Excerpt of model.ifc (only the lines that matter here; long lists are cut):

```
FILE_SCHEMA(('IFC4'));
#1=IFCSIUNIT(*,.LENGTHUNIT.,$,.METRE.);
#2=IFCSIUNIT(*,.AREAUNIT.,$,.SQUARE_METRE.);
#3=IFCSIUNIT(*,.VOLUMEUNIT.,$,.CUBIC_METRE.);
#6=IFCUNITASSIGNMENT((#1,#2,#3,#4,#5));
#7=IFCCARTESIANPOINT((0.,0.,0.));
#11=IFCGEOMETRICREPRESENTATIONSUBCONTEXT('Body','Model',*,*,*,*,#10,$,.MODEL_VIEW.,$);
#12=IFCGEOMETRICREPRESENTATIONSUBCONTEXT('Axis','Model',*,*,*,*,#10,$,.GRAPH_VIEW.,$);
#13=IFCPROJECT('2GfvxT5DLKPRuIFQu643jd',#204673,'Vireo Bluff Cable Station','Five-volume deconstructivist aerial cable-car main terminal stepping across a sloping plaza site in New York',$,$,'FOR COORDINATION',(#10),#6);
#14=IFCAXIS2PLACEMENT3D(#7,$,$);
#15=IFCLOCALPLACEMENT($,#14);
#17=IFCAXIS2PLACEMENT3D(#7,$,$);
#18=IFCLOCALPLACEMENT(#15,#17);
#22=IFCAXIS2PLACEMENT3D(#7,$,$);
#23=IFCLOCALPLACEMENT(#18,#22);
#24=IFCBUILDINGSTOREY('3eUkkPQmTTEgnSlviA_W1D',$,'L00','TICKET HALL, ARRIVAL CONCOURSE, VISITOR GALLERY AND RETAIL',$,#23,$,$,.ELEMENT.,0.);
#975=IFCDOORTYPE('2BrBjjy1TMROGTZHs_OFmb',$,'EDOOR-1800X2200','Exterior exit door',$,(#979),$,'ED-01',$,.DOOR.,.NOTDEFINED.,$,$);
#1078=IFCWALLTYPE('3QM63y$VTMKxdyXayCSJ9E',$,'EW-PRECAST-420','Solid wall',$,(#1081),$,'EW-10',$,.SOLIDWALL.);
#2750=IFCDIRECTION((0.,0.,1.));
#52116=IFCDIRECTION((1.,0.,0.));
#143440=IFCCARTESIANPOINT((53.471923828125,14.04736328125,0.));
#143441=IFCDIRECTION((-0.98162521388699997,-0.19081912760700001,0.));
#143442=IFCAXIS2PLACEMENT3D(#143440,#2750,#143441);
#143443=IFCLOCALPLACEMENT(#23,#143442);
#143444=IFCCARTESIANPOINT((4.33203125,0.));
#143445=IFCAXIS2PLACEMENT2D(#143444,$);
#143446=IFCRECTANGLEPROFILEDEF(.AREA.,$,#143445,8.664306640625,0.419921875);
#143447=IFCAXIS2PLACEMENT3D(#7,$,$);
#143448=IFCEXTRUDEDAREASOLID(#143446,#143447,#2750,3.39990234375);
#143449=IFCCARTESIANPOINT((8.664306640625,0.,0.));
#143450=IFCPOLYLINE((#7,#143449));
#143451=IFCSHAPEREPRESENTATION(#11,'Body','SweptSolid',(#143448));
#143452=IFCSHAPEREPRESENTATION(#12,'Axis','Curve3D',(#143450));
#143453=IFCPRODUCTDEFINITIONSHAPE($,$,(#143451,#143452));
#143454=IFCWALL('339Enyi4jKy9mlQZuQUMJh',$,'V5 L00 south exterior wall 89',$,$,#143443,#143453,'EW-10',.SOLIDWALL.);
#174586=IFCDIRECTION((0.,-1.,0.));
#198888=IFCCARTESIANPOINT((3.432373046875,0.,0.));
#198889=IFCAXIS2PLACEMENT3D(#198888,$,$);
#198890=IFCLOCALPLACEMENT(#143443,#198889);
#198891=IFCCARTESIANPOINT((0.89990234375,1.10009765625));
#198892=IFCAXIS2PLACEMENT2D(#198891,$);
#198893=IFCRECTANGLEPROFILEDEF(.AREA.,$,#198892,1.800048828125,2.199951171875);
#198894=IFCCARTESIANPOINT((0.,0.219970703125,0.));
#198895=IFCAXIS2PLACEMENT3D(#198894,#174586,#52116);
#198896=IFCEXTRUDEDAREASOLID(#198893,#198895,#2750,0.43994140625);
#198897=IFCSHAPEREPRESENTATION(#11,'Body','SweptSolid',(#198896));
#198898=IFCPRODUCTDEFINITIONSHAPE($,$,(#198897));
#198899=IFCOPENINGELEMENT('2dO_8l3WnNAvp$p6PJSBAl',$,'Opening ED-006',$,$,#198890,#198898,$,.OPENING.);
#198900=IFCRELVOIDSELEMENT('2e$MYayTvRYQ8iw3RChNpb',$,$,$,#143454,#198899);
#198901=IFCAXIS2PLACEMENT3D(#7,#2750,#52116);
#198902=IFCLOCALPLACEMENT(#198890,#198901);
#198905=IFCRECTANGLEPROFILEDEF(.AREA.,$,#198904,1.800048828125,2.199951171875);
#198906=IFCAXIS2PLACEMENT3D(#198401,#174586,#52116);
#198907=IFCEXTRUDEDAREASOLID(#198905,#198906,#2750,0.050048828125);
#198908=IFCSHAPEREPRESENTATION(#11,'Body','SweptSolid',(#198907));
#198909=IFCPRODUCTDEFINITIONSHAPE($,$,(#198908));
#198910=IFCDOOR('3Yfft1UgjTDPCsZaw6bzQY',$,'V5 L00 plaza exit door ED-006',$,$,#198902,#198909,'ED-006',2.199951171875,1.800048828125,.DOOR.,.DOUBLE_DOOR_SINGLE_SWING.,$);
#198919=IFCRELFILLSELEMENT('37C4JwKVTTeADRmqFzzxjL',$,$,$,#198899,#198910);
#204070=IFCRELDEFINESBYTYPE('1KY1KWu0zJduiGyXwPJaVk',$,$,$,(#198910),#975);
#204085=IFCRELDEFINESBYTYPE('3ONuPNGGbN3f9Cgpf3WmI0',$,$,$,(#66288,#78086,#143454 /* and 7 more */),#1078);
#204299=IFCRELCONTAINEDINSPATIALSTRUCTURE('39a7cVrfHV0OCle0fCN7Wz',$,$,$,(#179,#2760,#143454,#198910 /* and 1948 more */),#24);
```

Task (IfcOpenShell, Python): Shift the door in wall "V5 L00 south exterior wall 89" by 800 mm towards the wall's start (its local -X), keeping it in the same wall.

```python
import ifcopenshell
import ifcopenshell.api.geometry
import ifcopenshell.util.placement
import ifcopenshell.util.unit

model = ifcopenshell.open("model.ifc")
unit_scale = ifcopenshell.util.unit.calculate_unit_scale(model)

door = model.by_guid("3Yfft1UgjTDPCsZaw6bzQY")
opening = door.FillsVoids[0].RelatingOpeningElement
wall = opening.VoidsElements[0].RelatingBuildingElement

wall_matrix = ifcopenshell.util.placement.get_local_placement(wall.ObjectPlacement)
shift = wall_matrix[:3, 0] * -0.8 / unit_scale
before = ifcopenshell.util.placement.get_local_placement(door.ObjectPlacement)[:3, 3].copy()

# The door is placed relative to its opening, so it follows when the opening moves.
matrix = ifcopenshell.util.placement.get_local_placement(opening.ObjectPlacement)
matrix[:3, 3] += shift
ifcopenshell.api.geometry.edit_object_placement(
    model, product=opening, matrix=matrix, is_si=False, should_transform_children=True
)

after = ifcopenshell.util.placement.get_local_placement(door.ObjectPlacement)[:3, 3]
print("door moved by", (after - before).round(3) + 0.0)

model.write("model_edited.ifc")
```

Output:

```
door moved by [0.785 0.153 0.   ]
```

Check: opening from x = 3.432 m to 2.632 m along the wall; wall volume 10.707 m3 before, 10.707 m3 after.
